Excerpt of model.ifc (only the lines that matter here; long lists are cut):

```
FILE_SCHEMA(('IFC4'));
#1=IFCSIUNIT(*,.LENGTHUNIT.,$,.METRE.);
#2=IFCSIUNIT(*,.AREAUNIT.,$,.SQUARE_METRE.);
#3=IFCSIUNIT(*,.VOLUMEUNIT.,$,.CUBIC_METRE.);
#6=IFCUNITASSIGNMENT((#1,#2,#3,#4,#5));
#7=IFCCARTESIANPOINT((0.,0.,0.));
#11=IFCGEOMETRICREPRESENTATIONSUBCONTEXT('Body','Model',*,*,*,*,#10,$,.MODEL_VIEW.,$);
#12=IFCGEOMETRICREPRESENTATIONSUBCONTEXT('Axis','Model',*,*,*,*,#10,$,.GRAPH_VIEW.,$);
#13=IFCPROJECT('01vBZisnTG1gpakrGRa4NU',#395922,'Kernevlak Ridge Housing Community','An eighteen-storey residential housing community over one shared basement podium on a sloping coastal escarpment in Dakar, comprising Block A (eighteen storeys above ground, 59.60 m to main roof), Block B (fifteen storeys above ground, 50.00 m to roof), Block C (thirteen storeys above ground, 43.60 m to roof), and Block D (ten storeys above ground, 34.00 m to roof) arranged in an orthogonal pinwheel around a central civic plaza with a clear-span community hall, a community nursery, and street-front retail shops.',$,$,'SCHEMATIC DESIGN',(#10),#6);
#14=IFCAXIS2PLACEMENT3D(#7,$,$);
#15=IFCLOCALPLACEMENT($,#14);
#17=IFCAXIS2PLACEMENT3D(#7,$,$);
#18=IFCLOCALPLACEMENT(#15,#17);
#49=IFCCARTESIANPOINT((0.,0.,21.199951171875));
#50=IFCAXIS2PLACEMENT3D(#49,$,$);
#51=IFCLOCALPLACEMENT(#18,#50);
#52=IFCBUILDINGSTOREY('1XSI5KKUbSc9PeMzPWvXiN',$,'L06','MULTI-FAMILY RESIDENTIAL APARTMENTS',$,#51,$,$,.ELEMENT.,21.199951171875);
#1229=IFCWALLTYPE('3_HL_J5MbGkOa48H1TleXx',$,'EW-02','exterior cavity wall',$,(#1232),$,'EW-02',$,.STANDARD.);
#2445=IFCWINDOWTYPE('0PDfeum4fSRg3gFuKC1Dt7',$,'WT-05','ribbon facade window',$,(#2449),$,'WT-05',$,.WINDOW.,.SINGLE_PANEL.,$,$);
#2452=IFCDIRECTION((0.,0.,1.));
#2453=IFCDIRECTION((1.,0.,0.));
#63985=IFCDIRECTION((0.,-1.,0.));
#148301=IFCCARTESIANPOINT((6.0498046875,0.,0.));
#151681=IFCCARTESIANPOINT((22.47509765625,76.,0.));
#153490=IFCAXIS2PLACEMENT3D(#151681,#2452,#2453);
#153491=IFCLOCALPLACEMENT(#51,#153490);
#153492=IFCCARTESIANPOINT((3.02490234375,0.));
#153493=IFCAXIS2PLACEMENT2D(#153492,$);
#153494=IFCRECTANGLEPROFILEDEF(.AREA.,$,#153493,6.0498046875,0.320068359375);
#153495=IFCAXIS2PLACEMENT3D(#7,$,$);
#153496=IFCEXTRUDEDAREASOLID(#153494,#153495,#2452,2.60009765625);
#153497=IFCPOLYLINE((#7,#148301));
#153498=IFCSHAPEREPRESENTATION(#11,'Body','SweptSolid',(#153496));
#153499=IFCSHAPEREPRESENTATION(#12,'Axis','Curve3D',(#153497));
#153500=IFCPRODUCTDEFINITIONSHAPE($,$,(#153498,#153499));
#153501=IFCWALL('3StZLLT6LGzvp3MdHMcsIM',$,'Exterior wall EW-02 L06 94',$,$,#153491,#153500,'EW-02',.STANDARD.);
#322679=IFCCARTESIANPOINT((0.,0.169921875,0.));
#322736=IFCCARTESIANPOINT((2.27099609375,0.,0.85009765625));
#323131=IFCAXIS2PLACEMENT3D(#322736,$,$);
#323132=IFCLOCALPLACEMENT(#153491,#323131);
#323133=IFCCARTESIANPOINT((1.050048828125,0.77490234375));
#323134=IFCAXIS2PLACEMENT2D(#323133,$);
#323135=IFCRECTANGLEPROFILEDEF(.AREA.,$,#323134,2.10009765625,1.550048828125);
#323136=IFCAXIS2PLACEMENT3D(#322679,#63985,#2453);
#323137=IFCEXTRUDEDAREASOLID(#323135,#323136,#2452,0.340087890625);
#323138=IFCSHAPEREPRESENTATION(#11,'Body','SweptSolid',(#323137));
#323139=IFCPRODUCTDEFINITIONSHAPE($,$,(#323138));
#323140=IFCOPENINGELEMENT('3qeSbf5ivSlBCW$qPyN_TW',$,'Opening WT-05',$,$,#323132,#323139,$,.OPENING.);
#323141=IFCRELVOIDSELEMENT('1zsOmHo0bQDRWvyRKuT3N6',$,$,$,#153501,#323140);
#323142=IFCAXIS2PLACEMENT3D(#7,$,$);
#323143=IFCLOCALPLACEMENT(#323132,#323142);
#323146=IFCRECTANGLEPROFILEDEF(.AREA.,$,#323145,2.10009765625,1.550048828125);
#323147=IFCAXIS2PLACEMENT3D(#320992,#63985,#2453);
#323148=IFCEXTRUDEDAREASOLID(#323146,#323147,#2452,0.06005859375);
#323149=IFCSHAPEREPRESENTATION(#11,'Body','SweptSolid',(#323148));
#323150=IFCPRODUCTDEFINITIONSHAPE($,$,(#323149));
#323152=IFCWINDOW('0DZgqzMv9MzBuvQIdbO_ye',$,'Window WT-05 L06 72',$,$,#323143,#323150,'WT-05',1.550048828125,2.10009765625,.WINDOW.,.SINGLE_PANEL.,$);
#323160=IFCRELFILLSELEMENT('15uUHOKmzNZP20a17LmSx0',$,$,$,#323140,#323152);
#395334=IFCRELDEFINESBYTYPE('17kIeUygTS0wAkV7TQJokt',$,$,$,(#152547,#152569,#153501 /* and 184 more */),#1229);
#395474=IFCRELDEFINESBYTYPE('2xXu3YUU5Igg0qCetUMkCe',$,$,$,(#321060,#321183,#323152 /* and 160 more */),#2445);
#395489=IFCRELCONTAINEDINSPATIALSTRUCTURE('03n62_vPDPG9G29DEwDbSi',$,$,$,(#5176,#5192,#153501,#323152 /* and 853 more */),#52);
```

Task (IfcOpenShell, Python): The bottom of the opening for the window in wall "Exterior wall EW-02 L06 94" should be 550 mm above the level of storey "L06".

```python
import numpy as np
import ifcopenshell
import ifcopenshell.api.geometry
import ifcopenshell.geom
import ifcopenshell.util.element
import ifcopenshell.util.placement
import ifcopenshell.util.shape
import ifcopenshell.util.unit

model = ifcopenshell.open("model.ifc")
unit_scale = ifcopenshell.util.unit.calculate_unit_scale(model)

window = model.by_id(323152)
opening = window.FillsVoids[0].RelatingOpeningElement
storey = ifcopenshell.util.element.get_container(window, ifc_class="IfcBuildingStorey")
level = ifcopenshell.util.placement.get_local_placement(storey.ObjectPlacement)[2, 3]

# The opening's origin need not be at the sill, so measure its lowest point.
shape = ifcopenshell.geom.create_shape(ifcopenshell.geom.settings(), opening)
bottom = ifcopenshell.util.shape.get_shape_bottom_elevation(shape, shape.geometry) / unit_scale
dz = level + 0.55 - bottom

shift = np.array([0.0, 0.0, dz])
# The window is placed relative to its opening, so it follows when the opening moves.
matrix = ifcopenshell.util.placement.get_local_placement(opening.ObjectPlacement)
matrix[:3, 3] += shift
ifcopenshell.api.geometry.edit_object_placement(
    model, product=opening, matrix=matrix, is_si=False, should_transform_children=True
)

print(f"moved by {dz * unit_scale:+.3f} m")

model.write("model_v2.ifc")
```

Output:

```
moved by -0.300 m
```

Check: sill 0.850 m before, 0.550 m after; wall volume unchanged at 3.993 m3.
